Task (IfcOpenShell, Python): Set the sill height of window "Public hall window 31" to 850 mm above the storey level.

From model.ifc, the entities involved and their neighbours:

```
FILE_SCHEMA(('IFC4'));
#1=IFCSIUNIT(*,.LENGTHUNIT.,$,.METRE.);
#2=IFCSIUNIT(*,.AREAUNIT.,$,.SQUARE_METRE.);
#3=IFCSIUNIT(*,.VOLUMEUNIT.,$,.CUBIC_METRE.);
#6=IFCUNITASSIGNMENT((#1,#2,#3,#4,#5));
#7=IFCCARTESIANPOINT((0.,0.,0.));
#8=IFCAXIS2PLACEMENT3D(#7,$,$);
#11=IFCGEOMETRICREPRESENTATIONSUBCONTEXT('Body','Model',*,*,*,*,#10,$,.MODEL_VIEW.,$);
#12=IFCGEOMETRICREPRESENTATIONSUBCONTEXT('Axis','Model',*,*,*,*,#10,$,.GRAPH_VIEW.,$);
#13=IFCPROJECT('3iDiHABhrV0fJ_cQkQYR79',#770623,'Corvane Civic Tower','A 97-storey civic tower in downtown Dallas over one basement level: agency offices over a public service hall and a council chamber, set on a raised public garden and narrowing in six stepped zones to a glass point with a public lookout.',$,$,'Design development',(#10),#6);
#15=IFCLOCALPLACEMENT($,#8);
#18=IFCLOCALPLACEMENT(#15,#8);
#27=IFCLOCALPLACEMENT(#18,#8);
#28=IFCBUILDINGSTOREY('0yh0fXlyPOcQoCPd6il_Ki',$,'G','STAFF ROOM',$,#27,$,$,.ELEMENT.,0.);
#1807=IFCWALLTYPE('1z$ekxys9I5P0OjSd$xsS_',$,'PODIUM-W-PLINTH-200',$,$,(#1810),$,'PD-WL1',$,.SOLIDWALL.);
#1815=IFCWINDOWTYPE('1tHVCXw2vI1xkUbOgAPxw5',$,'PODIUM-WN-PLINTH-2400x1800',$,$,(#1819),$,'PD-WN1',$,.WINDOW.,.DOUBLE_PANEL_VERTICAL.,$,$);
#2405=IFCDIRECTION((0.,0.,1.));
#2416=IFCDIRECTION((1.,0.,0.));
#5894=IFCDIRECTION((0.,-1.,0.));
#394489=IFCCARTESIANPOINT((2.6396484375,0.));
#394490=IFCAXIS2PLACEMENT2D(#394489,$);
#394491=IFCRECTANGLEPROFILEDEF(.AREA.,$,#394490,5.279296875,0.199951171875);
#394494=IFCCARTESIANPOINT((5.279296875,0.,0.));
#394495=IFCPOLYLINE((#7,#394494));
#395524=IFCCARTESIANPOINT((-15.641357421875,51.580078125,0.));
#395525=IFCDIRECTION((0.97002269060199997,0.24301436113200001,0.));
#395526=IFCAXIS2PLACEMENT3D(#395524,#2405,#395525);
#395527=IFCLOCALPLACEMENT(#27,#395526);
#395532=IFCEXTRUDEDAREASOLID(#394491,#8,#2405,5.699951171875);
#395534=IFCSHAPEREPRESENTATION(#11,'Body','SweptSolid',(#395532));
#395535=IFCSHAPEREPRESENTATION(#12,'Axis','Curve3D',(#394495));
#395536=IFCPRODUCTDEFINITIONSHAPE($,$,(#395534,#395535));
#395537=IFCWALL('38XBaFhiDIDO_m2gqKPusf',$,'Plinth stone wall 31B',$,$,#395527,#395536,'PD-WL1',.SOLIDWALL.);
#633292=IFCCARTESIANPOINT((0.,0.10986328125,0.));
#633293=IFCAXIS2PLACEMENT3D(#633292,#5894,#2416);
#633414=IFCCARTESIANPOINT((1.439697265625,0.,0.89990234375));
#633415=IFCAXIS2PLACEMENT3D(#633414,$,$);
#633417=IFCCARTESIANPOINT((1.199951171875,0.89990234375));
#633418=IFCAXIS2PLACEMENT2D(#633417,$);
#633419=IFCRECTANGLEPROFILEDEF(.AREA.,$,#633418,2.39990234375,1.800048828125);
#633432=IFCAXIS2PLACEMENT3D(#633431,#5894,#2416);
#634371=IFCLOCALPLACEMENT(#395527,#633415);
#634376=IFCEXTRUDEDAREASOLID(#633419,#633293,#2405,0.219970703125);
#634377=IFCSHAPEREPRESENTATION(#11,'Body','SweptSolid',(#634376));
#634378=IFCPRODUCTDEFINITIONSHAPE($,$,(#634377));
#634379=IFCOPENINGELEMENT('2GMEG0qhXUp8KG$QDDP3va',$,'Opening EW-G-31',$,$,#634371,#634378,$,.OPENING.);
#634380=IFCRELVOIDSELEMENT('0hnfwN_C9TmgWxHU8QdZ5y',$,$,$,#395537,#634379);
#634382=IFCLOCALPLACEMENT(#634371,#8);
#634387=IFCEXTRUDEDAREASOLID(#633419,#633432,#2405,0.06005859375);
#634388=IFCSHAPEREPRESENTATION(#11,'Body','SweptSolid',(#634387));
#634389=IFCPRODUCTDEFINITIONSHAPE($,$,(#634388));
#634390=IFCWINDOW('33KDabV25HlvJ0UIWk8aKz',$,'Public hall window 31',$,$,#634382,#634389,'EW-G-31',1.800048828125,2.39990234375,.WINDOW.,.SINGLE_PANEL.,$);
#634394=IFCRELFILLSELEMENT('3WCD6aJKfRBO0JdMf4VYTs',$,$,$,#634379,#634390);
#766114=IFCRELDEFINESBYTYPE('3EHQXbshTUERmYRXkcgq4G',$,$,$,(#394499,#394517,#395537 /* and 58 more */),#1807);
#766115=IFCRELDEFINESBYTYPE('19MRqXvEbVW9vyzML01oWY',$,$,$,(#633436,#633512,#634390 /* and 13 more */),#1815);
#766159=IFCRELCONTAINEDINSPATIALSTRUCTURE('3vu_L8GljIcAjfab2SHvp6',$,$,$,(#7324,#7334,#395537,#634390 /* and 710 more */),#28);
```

```python
import numpy as np
import ifcopenshell
import ifcopenshell.api.geometry
import ifcopenshell.geom
import ifcopenshell.util.element
import ifcopenshell.util.placement
import ifcopenshell.util.shape
import ifcopenshell.util.unit

model = ifcopenshell.open("model.ifc")
unit_scale = ifcopenshell.util.unit.calculate_unit_scale(model)

window = model.by_guid("33KDabV25HlvJ0UIWk8aKz")
opening = window.FillsVoids[0].RelatingOpeningElement
storey = ifcopenshell.util.element.get_container(window, ifc_class="IfcBuildingStorey")
level = ifcopenshell.util.placement.get_local_placement(storey.ObjectPlacement)[2, 3]

# The opening's origin need not be at the sill, so measure its lowest point.
shape = ifcopenshell.geom.create_shape(ifcopenshell.geom.settings(), opening)
bottom = ifcopenshell.util.shape.get_shape_bottom_elevation(shape, shape.geometry) / unit_scale
dz = level + 0.85 - bottom

shift = np.array([0.0, 0.0, dz])
# The window is placed relative to its opening, so it follows when the opening moves.
matrix = ifcopenshell.util.placement.get_local_placement(opening.ObjectPlacement)
matrix[:3, 3] += shift
ifcopenshell.api.geometry.edit_object_placement(
    model, product=opening, matrix=matrix, is_si=False, should_transform_children=True
)

print(f"moved by {dz * unit_scale:+.3f} m")

model.write("model_v2.ifc")
```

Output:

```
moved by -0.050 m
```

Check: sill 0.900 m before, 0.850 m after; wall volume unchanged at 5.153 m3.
